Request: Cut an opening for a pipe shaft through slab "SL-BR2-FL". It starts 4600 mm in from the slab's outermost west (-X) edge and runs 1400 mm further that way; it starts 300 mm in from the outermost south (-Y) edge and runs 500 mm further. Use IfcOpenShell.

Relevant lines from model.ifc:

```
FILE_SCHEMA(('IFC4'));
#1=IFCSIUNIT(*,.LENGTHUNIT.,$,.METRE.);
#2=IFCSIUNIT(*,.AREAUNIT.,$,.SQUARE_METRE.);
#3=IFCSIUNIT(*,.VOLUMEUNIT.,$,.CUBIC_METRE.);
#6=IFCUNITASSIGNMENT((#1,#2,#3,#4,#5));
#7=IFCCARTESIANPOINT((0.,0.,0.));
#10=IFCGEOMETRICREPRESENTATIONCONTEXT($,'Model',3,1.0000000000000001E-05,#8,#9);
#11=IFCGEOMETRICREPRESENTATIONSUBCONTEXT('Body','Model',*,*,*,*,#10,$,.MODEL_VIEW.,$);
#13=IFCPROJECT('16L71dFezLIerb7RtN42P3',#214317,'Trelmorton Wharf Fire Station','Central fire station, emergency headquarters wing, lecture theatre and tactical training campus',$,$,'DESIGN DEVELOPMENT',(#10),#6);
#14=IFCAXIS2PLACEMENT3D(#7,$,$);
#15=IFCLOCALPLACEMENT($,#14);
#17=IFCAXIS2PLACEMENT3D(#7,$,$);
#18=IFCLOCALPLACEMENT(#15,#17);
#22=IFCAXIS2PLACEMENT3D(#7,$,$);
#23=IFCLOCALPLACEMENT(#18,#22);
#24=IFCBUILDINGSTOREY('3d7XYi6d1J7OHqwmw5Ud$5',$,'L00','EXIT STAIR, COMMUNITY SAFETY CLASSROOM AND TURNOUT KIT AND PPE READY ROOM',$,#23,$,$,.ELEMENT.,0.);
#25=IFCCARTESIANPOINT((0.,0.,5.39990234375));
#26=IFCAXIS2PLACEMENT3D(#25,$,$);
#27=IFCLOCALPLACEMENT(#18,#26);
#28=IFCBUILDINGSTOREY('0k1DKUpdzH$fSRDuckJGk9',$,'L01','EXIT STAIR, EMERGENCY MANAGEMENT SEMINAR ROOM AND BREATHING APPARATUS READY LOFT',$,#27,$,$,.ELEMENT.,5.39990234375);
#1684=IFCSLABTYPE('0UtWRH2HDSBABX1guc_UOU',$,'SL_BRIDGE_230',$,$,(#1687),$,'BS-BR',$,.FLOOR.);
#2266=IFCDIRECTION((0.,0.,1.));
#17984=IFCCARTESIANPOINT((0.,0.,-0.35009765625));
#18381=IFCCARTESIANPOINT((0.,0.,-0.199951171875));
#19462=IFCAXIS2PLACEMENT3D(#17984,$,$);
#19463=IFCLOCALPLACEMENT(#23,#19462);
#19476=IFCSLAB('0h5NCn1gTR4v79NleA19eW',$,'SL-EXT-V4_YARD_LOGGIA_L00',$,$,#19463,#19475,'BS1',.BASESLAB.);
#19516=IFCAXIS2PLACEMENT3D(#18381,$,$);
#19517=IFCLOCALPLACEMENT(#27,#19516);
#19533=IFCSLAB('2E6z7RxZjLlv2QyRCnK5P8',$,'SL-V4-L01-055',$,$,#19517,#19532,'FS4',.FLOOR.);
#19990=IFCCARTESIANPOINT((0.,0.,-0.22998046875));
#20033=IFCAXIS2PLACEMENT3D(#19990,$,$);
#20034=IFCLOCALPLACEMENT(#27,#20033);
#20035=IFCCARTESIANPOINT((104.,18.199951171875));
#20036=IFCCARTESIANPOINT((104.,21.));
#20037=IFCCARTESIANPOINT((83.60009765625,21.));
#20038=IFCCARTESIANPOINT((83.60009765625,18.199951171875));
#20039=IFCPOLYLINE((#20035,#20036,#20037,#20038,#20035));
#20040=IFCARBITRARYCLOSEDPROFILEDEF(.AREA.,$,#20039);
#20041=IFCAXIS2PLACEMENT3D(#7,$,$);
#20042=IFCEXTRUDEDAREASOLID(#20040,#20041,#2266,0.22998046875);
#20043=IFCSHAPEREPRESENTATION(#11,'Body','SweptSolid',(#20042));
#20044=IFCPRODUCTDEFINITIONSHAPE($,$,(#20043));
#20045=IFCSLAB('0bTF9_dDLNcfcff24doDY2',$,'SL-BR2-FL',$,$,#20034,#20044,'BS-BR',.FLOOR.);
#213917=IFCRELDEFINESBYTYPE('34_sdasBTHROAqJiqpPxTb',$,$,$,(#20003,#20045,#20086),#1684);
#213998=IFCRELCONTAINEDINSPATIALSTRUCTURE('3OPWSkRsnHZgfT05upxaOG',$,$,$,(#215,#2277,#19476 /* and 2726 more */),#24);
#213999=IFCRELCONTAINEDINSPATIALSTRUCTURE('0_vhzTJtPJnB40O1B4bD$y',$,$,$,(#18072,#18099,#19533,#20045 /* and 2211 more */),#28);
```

```python
import numpy as np
import ifcopenshell
import ifcopenshell.api.feature
import ifcopenshell.api.geometry
import ifcopenshell.api.root
import ifcopenshell.geom
import ifcopenshell.util.placement
import ifcopenshell.util.representation
import ifcopenshell.util.shape
import ifcopenshell.util.unit

model = ifcopenshell.open("model.ifc")
unit_scale = ifcopenshell.util.unit.calculate_unit_scale(model)
settings = ifcopenshell.geom.settings()


def volume(element):
    """Net volume in cubic metres, openings subtracted."""
    shape = ifcopenshell.geom.create_shape(settings, element)
    return ifcopenshell.util.shape.get_volume(shape.geometry)


slab = model.by_guid("0bTF9_dDLNcfcff24doDY2")
before = volume(slab)

# Extent in the slab's own axes, in metres. The edges named are its -X and -Y sides.
slab_shape = ifcopenshell.geom.create_shape(settings, slab)
vertices = ifcopenshell.util.shape.get_vertices(slab_shape.geometry)
x_min, y_min, bottom = vertices.min(axis=0)
top = vertices[:, 2].max()

opening = ifcopenshell.api.root.create_entity(model, ifc_class="IfcOpeningElement", name="Pipe shaft opening", predefined_type="OPENING")
context = ifcopenshell.util.representation.get_context(model, "Model", "Body", "MODEL_VIEW")
width, depth = 1.4, 0.5
outline = [(0.0, 0.0), (width, 0.0), (width, depth), (0.0, depth), (0.0, 0.0)]
# Overshoot both faces by 50 mm so the cut is clean.
shape = ifcopenshell.api.geometry.add_slab_representation(
    model, context=context, depth=top - bottom + 0.1, polyline=outline
)
ifcopenshell.api.geometry.assign_representation(model, product=opening, representation=shape)

matrix = ifcopenshell.util.placement.get_local_placement(slab.ObjectPlacement)
matrix[:, 3] = matrix @ np.append(np.array([x_min + 4.6, y_min + 0.3, bottom - 0.05]) / unit_scale, 1.0)
ifcopenshell.api.geometry.edit_object_placement(model, product=opening, matrix=matrix, is_si=False)
ifcopenshell.api.feature.add_feature(model, feature=opening, element=slab)

after = volume(slab)

print(f"slab volume {before:.3f} -> {after:.3f} m3")

model.write("model-out.ifc")
```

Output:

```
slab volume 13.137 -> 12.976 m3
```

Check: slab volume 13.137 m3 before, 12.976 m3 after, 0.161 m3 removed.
